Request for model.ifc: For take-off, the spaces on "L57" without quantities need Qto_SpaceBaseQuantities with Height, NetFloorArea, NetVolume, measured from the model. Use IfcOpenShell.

First a look at what the model holds.

```python
import ifcopenshell
import ifcopenshell.util.element
import ifcopenshell.util.unit

model = ifcopenshell.open("model.ifc")
print(model.schema)
for unit_type in ("LENGTHUNIT", "AREAUNIT", "VOLUMEUNIT"):
    print(unit_type, ifcopenshell.util.unit.calculate_unit_scale(model, unit_type))
storey = next(s for s in model.by_type("IfcBuildingStorey") if s.Name == "L57")
spaces = [e for e in ifcopenshell.util.element.get_decomposition(storey) if e.is_a("IfcSpace")]
for e in sorted(spaces, key=lambda e: e.id()):
    print(e.id(), e.is_a(), e.Name, list(ifcopenshell.util.element.get_psets(e, qtos_only=True)), sep=" | ")
```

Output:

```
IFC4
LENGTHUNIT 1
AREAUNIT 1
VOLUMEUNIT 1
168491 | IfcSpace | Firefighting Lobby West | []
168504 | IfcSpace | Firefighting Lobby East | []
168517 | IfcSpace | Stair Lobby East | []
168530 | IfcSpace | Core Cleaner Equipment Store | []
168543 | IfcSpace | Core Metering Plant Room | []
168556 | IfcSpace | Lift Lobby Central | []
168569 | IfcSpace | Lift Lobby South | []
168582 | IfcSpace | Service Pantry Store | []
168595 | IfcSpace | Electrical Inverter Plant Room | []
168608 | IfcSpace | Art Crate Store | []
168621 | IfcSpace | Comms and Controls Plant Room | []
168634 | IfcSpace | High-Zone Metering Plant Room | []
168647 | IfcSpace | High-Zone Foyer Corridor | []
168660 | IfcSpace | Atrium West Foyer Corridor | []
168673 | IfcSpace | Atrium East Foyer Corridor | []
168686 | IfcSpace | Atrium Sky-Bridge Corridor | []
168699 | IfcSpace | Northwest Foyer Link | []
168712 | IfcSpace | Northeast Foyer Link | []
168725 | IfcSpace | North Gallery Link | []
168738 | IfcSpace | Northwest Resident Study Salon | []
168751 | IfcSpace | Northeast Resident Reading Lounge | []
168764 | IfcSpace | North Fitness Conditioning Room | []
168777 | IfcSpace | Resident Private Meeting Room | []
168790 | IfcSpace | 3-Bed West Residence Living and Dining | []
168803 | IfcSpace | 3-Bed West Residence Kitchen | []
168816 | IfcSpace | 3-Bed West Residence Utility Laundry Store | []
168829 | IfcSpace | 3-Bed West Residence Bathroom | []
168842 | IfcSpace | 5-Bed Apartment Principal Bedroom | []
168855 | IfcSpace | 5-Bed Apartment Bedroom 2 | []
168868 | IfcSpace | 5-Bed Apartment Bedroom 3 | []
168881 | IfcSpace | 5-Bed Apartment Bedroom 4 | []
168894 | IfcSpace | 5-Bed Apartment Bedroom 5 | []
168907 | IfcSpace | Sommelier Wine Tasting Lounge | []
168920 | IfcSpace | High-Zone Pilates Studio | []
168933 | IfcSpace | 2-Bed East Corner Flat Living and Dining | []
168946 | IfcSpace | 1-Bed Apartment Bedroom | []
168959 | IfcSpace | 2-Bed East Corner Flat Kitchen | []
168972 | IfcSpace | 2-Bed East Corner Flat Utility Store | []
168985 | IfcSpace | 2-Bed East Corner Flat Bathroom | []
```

```python
import ifcopenshell
import ifcopenshell.api.pset
import ifcopenshell.geom
import ifcopenshell.util.element
import ifcopenshell.util.shape
import ifcopenshell.util.unit

model = ifcopenshell.open("model.ifc")
unit_scale = ifcopenshell.util.unit.calculate_unit_scale(model)
area_scale = ifcopenshell.util.unit.calculate_unit_scale(model, "AREAUNIT")
volume_scale = ifcopenshell.util.unit.calculate_unit_scale(model, "VOLUMEUNIT")
settings = ifcopenshell.geom.settings()

storey = next(s for s in model.by_type("IfcBuildingStorey") if s.Name == "L57")
spaces = [e for e in ifcopenshell.util.element.get_decomposition(storey) if e.is_a("IfcSpace")]

for e in sorted(spaces, key=lambda e: e.id()):
    if ifcopenshell.util.element.get_psets(e, qtos_only=True, should_inherit=False):
        continue
    # Geometry comes back in metres, in the element's own axes.
    shape = ifcopenshell.geom.create_shape(settings, e)
    values = {
        "Height": ifcopenshell.util.shape.get_z(shape.geometry) / unit_scale,
        "NetFloorArea": ifcopenshell.util.shape.get_footprint_area(shape.geometry) / area_scale,
        "NetVolume": ifcopenshell.util.shape.get_volume(shape.geometry) / volume_scale,
    }
    qto = ifcopenshell.api.pset.add_qto(model, product=e, name="Qto_SpaceBaseQuantities")
    ifcopenshell.api.pset.edit_qto(model, qto=qto, properties=values)
    print(e.id(), {k: round(v, 3) for k, v in values.items()})

model.write("model-out.ifc")
```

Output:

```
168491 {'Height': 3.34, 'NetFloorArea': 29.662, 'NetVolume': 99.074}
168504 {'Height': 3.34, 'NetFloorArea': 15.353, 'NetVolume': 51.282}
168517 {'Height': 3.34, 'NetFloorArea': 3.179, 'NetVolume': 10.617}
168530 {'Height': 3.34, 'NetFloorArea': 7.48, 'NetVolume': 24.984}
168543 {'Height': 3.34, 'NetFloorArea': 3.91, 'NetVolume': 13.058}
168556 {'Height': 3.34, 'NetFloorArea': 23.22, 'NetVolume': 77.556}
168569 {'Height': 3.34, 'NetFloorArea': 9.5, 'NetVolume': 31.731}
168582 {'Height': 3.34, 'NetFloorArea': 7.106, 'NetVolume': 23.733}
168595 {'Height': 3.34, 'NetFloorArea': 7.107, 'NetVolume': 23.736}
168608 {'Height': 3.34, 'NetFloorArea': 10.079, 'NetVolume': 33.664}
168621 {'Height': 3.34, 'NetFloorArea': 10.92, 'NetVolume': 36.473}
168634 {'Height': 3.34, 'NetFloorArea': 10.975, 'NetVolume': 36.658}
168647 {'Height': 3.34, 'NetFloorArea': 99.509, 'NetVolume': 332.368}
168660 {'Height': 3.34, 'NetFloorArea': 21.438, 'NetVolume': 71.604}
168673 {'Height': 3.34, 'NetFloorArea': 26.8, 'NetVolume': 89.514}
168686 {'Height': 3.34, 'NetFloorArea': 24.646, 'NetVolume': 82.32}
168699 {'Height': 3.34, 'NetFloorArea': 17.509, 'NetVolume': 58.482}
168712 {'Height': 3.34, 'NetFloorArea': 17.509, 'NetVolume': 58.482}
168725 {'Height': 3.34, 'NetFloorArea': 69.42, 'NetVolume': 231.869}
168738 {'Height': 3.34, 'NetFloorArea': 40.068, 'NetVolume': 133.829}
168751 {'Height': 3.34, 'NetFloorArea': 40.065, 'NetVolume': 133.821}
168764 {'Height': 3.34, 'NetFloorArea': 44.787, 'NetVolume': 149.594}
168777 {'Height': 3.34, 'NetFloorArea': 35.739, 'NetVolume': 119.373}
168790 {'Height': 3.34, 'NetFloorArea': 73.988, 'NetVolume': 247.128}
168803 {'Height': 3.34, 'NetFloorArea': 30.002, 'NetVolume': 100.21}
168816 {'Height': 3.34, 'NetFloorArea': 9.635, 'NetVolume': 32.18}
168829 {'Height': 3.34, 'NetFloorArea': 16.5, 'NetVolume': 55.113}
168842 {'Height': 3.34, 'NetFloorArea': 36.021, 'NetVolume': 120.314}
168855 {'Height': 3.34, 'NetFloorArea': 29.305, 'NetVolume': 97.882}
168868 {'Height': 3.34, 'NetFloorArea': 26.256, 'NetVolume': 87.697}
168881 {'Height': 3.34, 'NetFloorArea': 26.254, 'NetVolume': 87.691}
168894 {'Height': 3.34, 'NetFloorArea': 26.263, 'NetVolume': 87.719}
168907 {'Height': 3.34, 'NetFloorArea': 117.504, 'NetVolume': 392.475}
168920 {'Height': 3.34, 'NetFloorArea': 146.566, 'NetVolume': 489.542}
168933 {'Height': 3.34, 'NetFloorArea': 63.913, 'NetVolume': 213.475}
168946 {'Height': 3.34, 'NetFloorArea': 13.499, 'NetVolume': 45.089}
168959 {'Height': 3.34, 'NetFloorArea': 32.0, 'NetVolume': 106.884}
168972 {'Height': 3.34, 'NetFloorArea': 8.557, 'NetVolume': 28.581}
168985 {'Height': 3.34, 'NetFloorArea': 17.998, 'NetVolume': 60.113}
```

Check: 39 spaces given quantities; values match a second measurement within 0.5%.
